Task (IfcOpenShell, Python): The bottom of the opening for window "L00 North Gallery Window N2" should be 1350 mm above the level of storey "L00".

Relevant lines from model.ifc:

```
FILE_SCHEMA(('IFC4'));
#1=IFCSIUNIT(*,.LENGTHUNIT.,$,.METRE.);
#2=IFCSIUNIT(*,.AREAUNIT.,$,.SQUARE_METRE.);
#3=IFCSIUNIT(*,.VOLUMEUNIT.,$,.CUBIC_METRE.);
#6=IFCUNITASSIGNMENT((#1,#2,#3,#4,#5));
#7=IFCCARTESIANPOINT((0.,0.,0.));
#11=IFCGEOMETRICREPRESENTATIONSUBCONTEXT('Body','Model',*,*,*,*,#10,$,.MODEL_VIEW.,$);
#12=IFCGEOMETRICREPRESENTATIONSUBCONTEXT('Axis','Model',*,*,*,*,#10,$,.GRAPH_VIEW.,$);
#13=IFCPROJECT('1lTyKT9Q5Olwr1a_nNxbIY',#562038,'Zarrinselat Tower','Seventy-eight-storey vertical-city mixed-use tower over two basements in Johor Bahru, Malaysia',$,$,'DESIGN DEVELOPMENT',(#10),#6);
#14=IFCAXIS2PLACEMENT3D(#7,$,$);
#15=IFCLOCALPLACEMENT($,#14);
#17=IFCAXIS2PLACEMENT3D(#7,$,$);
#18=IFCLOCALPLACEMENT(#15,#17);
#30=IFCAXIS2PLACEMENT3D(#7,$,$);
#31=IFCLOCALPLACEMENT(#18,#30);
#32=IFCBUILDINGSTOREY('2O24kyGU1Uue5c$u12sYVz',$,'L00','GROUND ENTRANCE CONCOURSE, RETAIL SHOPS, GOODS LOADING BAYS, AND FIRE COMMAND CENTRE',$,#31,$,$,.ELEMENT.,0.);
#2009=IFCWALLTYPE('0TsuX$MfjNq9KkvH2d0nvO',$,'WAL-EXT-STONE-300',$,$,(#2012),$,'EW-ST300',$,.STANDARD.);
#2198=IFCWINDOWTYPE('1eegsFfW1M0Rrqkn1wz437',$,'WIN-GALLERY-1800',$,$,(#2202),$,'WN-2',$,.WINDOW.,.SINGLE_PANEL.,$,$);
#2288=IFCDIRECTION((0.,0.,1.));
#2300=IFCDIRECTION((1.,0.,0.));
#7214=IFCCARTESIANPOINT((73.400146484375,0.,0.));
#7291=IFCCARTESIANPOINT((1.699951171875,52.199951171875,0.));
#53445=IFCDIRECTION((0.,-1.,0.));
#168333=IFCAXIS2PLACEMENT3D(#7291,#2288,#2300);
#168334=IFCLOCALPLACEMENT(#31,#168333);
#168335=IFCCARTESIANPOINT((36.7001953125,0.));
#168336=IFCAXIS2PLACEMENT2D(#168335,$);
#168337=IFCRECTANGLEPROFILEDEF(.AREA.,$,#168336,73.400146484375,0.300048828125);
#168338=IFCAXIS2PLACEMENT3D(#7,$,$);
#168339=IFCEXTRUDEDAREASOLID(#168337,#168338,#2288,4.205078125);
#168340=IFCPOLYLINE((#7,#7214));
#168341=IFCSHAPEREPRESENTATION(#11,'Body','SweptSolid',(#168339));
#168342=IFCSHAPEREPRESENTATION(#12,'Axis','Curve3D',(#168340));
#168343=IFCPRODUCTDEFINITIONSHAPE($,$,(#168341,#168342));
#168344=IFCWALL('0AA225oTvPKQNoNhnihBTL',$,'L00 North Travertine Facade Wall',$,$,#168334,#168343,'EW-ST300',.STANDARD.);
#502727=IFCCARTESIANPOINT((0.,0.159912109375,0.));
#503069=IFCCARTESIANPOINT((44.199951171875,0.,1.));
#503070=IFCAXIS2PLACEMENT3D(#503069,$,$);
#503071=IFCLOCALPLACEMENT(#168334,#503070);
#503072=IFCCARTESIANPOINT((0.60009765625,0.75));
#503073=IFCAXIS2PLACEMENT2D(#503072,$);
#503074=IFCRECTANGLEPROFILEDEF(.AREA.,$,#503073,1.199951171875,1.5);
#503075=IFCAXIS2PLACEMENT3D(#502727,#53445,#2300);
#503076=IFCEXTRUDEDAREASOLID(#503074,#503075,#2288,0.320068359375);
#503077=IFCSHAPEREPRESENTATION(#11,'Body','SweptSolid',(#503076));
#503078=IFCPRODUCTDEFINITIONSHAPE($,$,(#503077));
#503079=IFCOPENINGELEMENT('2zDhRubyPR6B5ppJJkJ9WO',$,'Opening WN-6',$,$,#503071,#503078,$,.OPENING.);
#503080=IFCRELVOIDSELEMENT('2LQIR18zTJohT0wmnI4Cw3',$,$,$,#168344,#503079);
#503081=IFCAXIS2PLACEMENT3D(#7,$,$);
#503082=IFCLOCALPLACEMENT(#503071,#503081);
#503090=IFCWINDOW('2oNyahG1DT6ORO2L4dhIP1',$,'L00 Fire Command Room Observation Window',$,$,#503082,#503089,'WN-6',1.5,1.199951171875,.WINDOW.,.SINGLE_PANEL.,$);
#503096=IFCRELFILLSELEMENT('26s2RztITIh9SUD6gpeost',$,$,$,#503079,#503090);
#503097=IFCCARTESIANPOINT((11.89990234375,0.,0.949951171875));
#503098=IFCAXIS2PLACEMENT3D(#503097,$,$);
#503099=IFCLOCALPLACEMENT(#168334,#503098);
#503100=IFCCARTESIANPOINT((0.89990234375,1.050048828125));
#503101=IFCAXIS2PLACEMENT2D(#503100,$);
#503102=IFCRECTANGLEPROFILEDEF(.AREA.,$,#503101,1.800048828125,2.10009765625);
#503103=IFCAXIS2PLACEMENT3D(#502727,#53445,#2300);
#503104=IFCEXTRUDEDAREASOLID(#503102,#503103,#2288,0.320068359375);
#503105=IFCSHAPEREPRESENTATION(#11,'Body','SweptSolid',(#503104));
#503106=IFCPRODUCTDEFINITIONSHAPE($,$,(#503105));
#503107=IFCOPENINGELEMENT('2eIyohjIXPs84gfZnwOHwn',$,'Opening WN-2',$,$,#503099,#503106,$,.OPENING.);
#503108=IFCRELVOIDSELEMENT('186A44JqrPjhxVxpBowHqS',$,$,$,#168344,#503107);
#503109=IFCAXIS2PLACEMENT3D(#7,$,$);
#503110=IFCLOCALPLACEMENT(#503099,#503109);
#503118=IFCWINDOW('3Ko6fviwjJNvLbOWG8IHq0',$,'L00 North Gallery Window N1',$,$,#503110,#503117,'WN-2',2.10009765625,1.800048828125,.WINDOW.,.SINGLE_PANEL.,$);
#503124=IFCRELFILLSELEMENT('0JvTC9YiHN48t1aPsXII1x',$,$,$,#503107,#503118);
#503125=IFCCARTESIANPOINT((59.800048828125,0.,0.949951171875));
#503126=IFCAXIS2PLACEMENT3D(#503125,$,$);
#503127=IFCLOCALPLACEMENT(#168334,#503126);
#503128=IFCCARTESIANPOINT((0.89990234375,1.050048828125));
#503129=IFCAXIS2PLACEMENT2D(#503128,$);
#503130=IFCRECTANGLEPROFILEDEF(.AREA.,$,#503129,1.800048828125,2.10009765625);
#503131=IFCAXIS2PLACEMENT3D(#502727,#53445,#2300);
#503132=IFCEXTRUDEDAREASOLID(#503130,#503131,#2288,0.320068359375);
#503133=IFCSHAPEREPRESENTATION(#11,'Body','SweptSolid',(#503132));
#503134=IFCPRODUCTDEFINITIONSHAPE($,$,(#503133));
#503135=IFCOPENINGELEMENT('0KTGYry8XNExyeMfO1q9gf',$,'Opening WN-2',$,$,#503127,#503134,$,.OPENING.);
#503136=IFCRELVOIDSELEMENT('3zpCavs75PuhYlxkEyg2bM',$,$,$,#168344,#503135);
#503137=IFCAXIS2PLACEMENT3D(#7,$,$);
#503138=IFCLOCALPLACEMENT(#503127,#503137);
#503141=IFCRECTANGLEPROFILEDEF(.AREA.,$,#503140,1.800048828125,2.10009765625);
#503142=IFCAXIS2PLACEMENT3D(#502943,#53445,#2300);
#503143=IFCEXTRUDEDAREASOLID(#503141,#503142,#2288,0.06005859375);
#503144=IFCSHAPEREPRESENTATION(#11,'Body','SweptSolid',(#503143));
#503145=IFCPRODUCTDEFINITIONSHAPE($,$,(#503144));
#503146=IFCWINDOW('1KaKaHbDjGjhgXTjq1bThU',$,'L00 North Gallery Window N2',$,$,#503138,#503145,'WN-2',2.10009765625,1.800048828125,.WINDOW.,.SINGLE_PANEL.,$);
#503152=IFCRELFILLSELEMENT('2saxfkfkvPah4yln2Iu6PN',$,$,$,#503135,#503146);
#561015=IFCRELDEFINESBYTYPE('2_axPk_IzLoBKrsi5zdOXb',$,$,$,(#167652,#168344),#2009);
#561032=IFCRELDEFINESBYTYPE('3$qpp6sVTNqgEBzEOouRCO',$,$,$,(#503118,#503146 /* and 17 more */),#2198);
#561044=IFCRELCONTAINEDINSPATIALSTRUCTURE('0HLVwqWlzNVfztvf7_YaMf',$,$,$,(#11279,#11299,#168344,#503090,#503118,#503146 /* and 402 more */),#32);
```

```python
import numpy as np
import ifcopenshell
import ifcopenshell.api.geometry
import ifcopenshell.geom
import ifcopenshell.util.element
import ifcopenshell.util.placement
import ifcopenshell.util.shape
import ifcopenshell.util.unit

model = ifcopenshell.open("model.ifc")
unit_scale = ifcopenshell.util.unit.calculate_unit_scale(model)

window = model.by_guid("1KaKaHbDjGjhgXTjq1bThU")
opening = window.FillsVoids[0].RelatingOpeningElement
storey = ifcopenshell.util.element.get_container(window, ifc_class="IfcBuildingStorey")
level = ifcopenshell.util.placement.get_local_placement(storey.ObjectPlacement)[2, 3]

# The opening's origin need not be at the sill, so measure its lowest point.
shape = ifcopenshell.geom.create_shape(ifcopenshell.geom.settings(), opening)
bottom = ifcopenshell.util.shape.get_shape_bottom_elevation(shape, shape.geometry) / unit_scale
dz = level + 1.35 - bottom

shift = np.array([0.0, 0.0, dz])
# The window is placed relative to its opening, so it follows when the opening moves.
matrix = ifcopenshell.util.placement.get_local_placement(opening.ObjectPlacement)
matrix[:3, 3] += shift
ifcopenshell.api.geometry.edit_object_placement(
    model, product=opening, matrix=matrix, is_si=False, should_transform_children=True
)

print(f"moved by {dz * unit_scale:+.3f} m")

model.write("model-out.ifc")
```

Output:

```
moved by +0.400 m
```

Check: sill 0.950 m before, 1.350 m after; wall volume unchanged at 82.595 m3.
